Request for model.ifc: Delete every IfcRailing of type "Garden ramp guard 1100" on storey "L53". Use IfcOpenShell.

First a look at what the model holds.

```python
import ifcopenshell
import ifcopenshell.util.element

model = ifcopenshell.open("model.ifc")
print(model.schema)
storey = next(s for s in model.by_type("IfcBuildingStorey") if s.Name == "L53")
railings = [e for e in ifcopenshell.util.element.get_decomposition(storey) if e.is_a("IfcRailing")]
seen = {}
for e in railings:
    element_type = ifcopenshell.util.element.get_type(e)
    name = element_type.Name if element_type not in (None, e) else None
    seen[name] = seen.get(name, 0) + 1
for name, count in sorted(seen.items(), key=str):
    print(count, "x", name)
```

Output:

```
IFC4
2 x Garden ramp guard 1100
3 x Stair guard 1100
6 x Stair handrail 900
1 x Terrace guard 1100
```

```python
import ifcopenshell
import ifcopenshell.api.root
import ifcopenshell.util.element

model = ifcopenshell.open("model.ifc")

storey = next(s for s in model.by_type("IfcBuildingStorey") if s.Name == "L53")
railings = [e for e in ifcopenshell.util.element.get_decomposition(storey) if e.is_a("IfcRailing")]
targets = [e for e in railings if (t := ifcopenshell.util.element.get_type(e)) not in (None, e) and t.Name == "Garden ramp guard 1100"]

for e in targets:
    ifcopenshell.api.root.remove_product(model, product=e)
print(len(targets), "removed")

model.write("model_v2.ifc")
```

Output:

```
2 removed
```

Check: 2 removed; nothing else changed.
